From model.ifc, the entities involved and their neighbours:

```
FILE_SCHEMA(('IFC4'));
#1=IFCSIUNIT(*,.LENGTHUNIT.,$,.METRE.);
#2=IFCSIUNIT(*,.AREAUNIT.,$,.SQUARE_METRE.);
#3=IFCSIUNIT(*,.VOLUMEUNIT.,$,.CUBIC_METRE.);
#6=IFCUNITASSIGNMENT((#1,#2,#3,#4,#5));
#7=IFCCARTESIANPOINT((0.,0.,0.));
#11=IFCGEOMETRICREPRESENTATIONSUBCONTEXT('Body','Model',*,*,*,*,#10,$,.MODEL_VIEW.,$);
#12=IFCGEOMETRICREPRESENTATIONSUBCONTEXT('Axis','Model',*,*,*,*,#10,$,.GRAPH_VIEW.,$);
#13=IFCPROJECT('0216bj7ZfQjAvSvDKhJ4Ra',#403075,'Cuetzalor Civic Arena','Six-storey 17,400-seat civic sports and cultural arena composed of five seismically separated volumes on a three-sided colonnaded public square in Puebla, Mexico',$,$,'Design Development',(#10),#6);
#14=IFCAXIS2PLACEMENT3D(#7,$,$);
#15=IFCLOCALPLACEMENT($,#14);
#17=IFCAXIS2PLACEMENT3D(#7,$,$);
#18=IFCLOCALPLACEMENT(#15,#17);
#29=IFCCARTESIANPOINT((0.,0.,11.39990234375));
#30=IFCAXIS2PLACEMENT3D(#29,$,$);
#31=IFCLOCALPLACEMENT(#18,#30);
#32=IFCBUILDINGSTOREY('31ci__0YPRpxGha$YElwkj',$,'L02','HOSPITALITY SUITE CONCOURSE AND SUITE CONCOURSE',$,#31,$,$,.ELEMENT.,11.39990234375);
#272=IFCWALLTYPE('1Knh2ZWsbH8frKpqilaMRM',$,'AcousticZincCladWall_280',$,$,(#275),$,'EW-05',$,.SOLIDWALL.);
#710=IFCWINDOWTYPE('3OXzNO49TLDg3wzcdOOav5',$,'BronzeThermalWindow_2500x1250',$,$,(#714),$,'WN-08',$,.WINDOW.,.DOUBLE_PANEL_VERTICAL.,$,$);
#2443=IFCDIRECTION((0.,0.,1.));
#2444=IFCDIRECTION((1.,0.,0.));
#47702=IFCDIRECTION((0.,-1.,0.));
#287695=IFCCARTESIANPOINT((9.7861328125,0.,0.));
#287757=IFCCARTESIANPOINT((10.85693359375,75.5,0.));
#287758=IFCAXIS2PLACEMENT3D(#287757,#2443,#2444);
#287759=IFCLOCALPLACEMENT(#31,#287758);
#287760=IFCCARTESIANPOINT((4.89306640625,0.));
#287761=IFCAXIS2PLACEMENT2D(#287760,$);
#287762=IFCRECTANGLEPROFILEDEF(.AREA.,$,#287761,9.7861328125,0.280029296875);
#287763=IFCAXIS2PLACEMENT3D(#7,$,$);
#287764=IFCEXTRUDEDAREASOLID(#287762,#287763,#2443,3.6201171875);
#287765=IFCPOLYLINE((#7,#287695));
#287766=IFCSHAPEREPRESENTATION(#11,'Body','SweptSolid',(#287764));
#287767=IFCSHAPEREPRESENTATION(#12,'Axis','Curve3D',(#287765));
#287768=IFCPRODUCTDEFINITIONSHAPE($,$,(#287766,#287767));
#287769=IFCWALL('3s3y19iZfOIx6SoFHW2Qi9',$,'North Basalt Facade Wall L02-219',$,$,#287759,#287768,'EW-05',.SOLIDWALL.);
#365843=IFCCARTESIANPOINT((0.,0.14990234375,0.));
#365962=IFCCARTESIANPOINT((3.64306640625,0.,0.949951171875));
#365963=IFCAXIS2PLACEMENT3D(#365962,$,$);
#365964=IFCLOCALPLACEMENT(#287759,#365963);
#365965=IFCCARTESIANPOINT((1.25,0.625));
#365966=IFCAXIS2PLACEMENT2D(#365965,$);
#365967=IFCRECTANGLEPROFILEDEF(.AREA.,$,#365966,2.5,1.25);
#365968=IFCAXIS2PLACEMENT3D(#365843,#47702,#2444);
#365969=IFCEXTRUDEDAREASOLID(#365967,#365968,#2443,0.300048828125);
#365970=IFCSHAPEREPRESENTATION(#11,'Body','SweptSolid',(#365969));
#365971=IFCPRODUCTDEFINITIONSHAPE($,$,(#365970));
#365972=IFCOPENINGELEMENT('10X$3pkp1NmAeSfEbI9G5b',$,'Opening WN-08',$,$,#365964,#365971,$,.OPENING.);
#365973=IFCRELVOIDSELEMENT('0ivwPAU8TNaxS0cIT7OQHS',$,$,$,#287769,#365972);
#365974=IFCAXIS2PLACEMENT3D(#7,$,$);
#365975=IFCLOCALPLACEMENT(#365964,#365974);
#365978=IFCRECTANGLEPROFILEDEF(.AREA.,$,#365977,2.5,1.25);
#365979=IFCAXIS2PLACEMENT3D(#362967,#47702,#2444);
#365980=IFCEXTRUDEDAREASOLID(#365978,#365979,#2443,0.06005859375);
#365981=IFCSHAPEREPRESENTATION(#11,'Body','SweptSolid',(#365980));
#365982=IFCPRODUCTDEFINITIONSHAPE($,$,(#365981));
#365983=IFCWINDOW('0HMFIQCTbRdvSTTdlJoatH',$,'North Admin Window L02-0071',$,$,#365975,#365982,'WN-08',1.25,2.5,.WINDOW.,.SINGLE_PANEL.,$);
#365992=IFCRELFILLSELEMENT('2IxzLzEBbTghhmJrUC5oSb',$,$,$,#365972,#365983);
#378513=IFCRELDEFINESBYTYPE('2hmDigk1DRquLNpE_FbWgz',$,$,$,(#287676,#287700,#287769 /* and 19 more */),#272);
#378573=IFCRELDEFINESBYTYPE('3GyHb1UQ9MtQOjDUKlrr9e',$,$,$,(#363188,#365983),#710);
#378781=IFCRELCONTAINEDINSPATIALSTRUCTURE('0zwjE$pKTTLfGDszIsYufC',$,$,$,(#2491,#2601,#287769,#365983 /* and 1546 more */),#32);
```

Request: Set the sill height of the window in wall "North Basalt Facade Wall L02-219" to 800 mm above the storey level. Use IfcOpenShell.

```python
import numpy as np
import ifcopenshell
import ifcopenshell.api.geometry
import ifcopenshell.geom
import ifcopenshell.util.element
import ifcopenshell.util.placement
import ifcopenshell.util.shape
import ifcopenshell.util.unit

model = ifcopenshell.open("model.ifc")
unit_scale = ifcopenshell.util.unit.calculate_unit_scale(model)

window = model.by_id(365983)
opening = window.FillsVoids[0].RelatingOpeningElement
storey = ifcopenshell.util.element.get_container(window, ifc_class="IfcBuildingStorey")
level = ifcopenshell.util.placement.get_local_placement(storey.ObjectPlacement)[2, 3]

# The opening's origin need not be at the sill, so measure its lowest point.
shape = ifcopenshell.geom.create_shape(ifcopenshell.geom.settings(), opening)
bottom = ifcopenshell.util.shape.get_shape_bottom_elevation(shape, shape.geometry) / unit_scale
dz = level + 0.8 / unit_scale - bottom

shift = np.array([0.0, 0.0, dz])
# The window is placed relative to its opening, so it follows when the opening moves.
matrix = ifcopenshell.util.placement.get_local_placement(opening.ObjectPlacement)
matrix[:3, 3] += shift
ifcopenshell.api.geometry.edit_object_placement(
    model, product=opening, matrix=matrix, is_si=False, should_transform_children=True
)

print(f"moved by {dz * unit_scale:+.3f} m")

model.write("model-out.ifc")
```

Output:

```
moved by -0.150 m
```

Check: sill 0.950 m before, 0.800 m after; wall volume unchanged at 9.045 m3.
